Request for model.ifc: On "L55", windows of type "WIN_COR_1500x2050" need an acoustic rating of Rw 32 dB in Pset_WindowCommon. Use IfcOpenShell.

First a look at what the model holds.

```python
import ifcopenshell
import ifcopenshell.util.element

model = ifcopenshell.open("model.ifc")
print(model.schema)
storey = next(s for s in model.by_type("IfcBuildingStorey") if s.Name == "L55")
windows = [e for e in ifcopenshell.util.element.get_decomposition(storey) if e.is_a("IfcWindow")]
seen = {}
for e in windows:
    element_type = ifcopenshell.util.element.get_type(e)
    key = (element_type.Name if element_type != e and element_type else None, ifcopenshell.util.element.get_pset(e, "Pset_WindowCommon", "AcousticRating"))
    seen[key] = seen.get(key, 0) + 1
for (name, value), count in sorted(seen.items(), key=str):
    print(count, "x", name, "|", value)
```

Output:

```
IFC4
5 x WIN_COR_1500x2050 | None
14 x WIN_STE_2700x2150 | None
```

```python
import ifcopenshell
import ifcopenshell.api.pset
import ifcopenshell.util.element

model = ifcopenshell.open("model.ifc")

storey = next(s for s in model.by_type("IfcBuildingStorey") if s.Name == "L55")
windows = [e for e in ifcopenshell.util.element.get_decomposition(storey) if e.is_a("IfcWindow")]

count = 0
for e in windows:
    element_type = ifcopenshell.util.element.get_type(e)
    if element_type in (None, e) or element_type.Name != "WIN_COR_1500x2050":
        continue
    found = ifcopenshell.util.element.get_pset(e, "Pset_WindowCommon", should_inherit=False)
    if found:
        pset = model.by_id(found["id"])
        if len(ifcopenshell.util.element.get_elements_by_pset(pset)) > 1:
            pset = ifcopenshell.api.pset.unshare_pset(model, products=[e], pset=pset)[0]
    else:
        pset = ifcopenshell.api.pset.add_pset(model, product=e, name="Pset_WindowCommon")
    ifcopenshell.api.pset.edit_pset(model, pset=pset, properties={"AcousticRating": "Rw 32 dB"})
    count += 1

print(count, "windows updated")

model.write("model-out.ifc")
```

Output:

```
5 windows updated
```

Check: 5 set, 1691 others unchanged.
